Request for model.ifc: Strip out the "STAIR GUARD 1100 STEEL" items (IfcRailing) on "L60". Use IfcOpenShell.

First a look at what the model holds.

```python
import ifcopenshell
import ifcopenshell.util.element

model = ifcopenshell.open("model.ifc")
print(model.schema)
storey = next(s for s in model.by_type("IfcBuildingStorey") if s.Name == "L60")
railings = [e for e in ifcopenshell.util.element.get_decomposition(storey) if e.is_a("IfcRailing")]
seen = {}
for e in railings:
    element_type = ifcopenshell.util.element.get_type(e)
    name = element_type.Name if element_type not in (None, e) else None
    seen[name] = seen.get(name, 0) + 1
for name, count in sorted(seen.items(), key=str):
    print(count, "x", name)
```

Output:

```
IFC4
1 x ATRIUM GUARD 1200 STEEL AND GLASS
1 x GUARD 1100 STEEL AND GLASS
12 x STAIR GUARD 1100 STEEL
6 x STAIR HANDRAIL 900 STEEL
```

```python
import ifcopenshell
import ifcopenshell.api.root
import ifcopenshell.util.element

model = ifcopenshell.open("model.ifc")

storey = next(s for s in model.by_type("IfcBuildingStorey") if s.Name == "L60")
railings = [e for e in ifcopenshell.util.element.get_decomposition(storey) if e.is_a("IfcRailing")]
targets = [e for e in railings if (t := ifcopenshell.util.element.get_type(e)) not in (None, e) and t.Name == "STAIR GUARD 1100 STEEL"]

for e in targets:
    ifcopenshell.api.root.remove_product(model, product=e)
print(len(targets), "removed")

model.write("model_v2.ifc")
```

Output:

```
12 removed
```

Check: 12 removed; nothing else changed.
